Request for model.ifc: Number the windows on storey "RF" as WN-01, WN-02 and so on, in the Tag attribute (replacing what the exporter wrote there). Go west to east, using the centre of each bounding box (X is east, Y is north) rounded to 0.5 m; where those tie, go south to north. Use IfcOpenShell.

First a look at what the model holds.

```python
import ifcopenshell
import ifcopenshell.util.element
import ifcopenshell.util.placement

model = ifcopenshell.open("model.ifc")
print(model.schema)
storey = next(s for s in model.by_type("IfcBuildingStorey") if s.Name == "RF")
windows = [e for e in ifcopenshell.util.element.get_decomposition(storey) if e.is_a("IfcWindow")]
for e in sorted(windows, key=lambda e: e.id()):
    origin = ifcopenshell.util.placement.get_local_placement(e.ObjectPlacement)[:3, 3]
    print(e.id(), e.Tag, e.Name, origin.round(2) + 0.0, sep=" | ")
```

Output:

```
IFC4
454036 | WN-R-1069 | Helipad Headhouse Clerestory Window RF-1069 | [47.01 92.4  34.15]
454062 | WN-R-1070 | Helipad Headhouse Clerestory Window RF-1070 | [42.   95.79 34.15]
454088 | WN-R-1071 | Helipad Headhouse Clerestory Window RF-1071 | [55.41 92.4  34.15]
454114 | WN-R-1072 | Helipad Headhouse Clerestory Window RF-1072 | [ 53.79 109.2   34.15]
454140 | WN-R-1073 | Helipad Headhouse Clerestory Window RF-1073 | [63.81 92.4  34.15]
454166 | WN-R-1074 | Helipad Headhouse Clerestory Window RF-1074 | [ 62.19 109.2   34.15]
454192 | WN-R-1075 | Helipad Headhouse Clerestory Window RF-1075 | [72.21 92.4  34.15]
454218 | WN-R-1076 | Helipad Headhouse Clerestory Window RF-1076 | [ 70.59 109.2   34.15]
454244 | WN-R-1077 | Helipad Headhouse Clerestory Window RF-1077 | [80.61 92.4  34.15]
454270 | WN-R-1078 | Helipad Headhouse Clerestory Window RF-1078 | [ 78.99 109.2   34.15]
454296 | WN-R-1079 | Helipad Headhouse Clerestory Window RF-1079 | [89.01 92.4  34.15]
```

```python
import ifcopenshell
import ifcopenshell.geom
import ifcopenshell.util.element
import ifcopenshell.util.shape

model = ifcopenshell.open("model.ifc")
settings = ifcopenshell.geom.settings()
settings.set("use-world-coords", True)


def centre(element):
    shape = ifcopenshell.geom.create_shape(settings, element)
    return ifcopenshell.util.shape.get_bbox_centroid(shape.geometry)


storey = next(s for s in model.by_type("IfcBuildingStorey") if s.Name == "RF")
windows = [e for e in ifcopenshell.util.element.get_decomposition(storey) if e.is_a("IfcWindow")]

# Insertion points can sit at a corner or the storey origin, so sort by the geometry (in metres).
centres = {e: centre(e) for e in windows}
windows.sort(key=lambda e: (round(centres[e][0] / 0.5), centres[e][1]))

for i, e in enumerate(windows, start=1):
    number = f"WN-{i:02d}"
    e.Tag = number
    print(e.id(), number)

model.write("model_updated.ifc")
```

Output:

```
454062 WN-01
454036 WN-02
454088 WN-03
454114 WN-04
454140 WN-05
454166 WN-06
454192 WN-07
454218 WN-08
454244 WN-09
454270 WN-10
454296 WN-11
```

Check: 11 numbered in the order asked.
